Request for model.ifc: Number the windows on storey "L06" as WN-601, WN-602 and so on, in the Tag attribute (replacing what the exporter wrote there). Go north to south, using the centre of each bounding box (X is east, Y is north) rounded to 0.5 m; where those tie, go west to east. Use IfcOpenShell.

First a look at what the model holds.

```python
import ifcopenshell
import ifcopenshell.util.element
import ifcopenshell.util.placement

model = ifcopenshell.open("model.ifc")
print(model.schema)
storey = next(s for s in model.by_type("IfcBuildingStorey") if s.Name == "L06")
windows = [e for e in ifcopenshell.util.element.get_decomposition(storey) if e.is_a("IfcWindow")]
for e in sorted(windows, key=lambda e: e.id()):
    origin = ifcopenshell.util.placement.get_local_placement(e.ObjectPlacement)[:3, 3]
    print(e.id(), e.Tag, e.Name, origin.round(2) + 0.0, sep=" | ")
```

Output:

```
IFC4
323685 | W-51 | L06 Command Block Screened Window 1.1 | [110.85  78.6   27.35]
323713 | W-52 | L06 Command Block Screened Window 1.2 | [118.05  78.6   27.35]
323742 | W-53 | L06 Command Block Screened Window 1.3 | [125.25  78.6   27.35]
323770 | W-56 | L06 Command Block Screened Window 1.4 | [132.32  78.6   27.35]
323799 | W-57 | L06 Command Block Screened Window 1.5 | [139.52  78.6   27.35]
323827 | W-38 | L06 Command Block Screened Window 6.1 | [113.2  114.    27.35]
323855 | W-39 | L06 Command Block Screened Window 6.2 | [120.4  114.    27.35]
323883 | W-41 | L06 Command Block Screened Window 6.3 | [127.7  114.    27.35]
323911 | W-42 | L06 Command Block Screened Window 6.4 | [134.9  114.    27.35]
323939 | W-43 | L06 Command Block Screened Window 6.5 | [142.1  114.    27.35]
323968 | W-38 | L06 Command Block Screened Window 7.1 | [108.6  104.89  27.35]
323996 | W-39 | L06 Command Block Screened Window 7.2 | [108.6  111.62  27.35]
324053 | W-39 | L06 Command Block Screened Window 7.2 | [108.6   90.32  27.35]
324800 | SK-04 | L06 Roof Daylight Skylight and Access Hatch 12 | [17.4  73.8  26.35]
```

```python
import ifcopenshell
import ifcopenshell.geom
import ifcopenshell.util.element
import ifcopenshell.util.shape

model = ifcopenshell.open("model.ifc")
settings = ifcopenshell.geom.settings()
settings.set("use-world-coords", True)


def centre(element):
    shape = ifcopenshell.geom.create_shape(settings, element)
    return ifcopenshell.util.shape.get_bbox_centroid(shape.geometry)


storey = next(s for s in model.by_type("IfcBuildingStorey") if s.Name == "L06")
windows = [e for e in ifcopenshell.util.element.get_decomposition(storey) if e.is_a("IfcWindow")]

# Insertion points can sit at a corner or the storey origin, so sort by the geometry (in metres).
centres = {e: centre(e) for e in windows}
windows.sort(key=lambda e: (-round(centres[e][1] / 0.5), centres[e][0]))

for i, e in enumerate(windows, start=1):
    number = f"WN-6{i:02d}"
    e.Tag = number
    print(e.id(), number)

model.write("model_updated.ifc")
```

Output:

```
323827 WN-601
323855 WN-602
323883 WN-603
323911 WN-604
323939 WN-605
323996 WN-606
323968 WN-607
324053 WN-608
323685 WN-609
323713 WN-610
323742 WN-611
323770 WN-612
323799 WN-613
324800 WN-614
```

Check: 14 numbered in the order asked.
